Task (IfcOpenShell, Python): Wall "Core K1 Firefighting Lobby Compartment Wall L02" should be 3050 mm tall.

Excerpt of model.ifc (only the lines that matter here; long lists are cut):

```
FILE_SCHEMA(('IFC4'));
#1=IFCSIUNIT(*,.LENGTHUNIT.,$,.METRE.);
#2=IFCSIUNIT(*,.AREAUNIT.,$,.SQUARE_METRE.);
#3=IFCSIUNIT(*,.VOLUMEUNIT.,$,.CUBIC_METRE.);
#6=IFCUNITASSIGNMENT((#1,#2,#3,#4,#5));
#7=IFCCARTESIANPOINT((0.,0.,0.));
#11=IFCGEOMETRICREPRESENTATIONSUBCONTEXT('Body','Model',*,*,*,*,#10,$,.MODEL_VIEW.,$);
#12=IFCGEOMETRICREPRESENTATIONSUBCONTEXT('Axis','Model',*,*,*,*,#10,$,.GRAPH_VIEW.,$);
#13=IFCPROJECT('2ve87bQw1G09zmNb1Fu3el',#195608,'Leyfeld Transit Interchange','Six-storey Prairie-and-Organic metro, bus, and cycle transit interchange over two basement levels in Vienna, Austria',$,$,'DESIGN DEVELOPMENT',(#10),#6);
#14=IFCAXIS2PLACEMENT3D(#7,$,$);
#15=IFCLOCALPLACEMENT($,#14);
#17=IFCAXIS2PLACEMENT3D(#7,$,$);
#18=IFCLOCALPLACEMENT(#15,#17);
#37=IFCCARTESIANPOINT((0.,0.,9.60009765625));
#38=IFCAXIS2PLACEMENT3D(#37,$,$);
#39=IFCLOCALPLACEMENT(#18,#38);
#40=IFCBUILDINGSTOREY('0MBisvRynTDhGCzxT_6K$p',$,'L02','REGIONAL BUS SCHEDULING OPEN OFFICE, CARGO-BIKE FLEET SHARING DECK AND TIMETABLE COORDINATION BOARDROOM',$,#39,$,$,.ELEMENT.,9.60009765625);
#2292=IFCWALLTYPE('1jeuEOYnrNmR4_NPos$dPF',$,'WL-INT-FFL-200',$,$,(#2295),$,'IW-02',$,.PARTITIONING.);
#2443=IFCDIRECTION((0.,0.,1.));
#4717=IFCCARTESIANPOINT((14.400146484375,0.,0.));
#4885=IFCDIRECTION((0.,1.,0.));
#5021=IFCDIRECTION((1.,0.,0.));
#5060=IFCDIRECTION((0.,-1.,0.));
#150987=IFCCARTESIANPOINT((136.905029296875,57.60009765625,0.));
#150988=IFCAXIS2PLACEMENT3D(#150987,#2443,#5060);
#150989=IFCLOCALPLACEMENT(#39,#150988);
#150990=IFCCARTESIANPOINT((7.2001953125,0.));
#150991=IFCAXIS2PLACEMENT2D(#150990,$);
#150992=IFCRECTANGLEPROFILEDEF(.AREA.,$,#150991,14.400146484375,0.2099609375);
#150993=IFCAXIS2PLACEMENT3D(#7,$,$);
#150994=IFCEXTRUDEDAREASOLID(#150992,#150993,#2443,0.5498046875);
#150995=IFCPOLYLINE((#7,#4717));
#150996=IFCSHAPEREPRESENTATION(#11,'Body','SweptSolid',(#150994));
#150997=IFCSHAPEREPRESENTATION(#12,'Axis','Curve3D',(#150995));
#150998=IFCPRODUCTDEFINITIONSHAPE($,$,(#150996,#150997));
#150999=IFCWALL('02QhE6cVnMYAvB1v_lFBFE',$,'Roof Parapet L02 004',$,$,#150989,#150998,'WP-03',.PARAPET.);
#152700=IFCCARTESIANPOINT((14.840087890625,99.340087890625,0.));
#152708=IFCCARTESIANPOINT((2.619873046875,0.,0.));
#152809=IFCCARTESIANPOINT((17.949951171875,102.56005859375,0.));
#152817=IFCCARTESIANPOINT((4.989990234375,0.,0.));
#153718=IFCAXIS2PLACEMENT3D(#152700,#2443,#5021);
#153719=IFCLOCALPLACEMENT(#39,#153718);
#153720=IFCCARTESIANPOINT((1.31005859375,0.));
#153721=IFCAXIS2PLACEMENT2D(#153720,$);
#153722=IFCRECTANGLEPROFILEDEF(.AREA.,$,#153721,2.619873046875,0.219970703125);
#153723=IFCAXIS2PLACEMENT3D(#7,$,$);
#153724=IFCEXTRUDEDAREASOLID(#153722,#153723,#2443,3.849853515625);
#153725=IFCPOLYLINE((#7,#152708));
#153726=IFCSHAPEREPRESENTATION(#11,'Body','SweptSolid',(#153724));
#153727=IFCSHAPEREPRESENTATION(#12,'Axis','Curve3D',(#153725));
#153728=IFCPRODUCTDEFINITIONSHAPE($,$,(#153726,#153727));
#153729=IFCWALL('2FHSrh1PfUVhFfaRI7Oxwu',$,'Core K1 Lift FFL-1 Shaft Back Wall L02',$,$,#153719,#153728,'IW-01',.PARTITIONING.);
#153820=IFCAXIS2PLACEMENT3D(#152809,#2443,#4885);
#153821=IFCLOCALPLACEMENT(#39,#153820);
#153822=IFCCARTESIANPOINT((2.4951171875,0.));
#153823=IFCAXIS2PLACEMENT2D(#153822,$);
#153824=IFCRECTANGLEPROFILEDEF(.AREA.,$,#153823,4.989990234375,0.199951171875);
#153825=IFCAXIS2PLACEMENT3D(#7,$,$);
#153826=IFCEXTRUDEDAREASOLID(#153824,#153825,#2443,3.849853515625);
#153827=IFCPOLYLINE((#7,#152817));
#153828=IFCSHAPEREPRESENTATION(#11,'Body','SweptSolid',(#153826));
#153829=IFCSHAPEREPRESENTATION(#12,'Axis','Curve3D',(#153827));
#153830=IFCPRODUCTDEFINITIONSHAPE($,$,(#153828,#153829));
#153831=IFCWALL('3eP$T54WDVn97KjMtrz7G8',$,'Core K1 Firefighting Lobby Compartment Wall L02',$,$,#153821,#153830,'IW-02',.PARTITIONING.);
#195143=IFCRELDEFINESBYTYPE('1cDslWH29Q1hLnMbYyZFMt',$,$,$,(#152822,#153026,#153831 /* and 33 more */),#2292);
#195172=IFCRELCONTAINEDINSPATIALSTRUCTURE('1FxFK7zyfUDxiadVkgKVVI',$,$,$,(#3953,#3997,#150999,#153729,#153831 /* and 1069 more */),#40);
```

```python
import ifcopenshell
import ifcopenshell.geom
import ifcopenshell.util.representation
import ifcopenshell.util.shape

model = ifcopenshell.open("model.ifc")
settings = ifcopenshell.geom.settings()


def volume(element):
    """Net volume in cubic metres, openings subtracted."""
    shape = ifcopenshell.geom.create_shape(settings, element)
    return ifcopenshell.util.shape.get_volume(shape.geometry)


wall = model.by_guid("3eP$T54WDVn97KjMtrz7G8")
before = volume(wall)

body = ifcopenshell.util.representation.get_representation(wall, "Model", "Body")
solid = body.Items[0]
old_height = solid.Depth
solid.Depth = 3.05
after = volume(wall)

print(f"height {old_height:g} -> {solid.Depth:g}, volume {before:.3f} -> {after:.3f} m3")

model.write("model_updated.ifc")
```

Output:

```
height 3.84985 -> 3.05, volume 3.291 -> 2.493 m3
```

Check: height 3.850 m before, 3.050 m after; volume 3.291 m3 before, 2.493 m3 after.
